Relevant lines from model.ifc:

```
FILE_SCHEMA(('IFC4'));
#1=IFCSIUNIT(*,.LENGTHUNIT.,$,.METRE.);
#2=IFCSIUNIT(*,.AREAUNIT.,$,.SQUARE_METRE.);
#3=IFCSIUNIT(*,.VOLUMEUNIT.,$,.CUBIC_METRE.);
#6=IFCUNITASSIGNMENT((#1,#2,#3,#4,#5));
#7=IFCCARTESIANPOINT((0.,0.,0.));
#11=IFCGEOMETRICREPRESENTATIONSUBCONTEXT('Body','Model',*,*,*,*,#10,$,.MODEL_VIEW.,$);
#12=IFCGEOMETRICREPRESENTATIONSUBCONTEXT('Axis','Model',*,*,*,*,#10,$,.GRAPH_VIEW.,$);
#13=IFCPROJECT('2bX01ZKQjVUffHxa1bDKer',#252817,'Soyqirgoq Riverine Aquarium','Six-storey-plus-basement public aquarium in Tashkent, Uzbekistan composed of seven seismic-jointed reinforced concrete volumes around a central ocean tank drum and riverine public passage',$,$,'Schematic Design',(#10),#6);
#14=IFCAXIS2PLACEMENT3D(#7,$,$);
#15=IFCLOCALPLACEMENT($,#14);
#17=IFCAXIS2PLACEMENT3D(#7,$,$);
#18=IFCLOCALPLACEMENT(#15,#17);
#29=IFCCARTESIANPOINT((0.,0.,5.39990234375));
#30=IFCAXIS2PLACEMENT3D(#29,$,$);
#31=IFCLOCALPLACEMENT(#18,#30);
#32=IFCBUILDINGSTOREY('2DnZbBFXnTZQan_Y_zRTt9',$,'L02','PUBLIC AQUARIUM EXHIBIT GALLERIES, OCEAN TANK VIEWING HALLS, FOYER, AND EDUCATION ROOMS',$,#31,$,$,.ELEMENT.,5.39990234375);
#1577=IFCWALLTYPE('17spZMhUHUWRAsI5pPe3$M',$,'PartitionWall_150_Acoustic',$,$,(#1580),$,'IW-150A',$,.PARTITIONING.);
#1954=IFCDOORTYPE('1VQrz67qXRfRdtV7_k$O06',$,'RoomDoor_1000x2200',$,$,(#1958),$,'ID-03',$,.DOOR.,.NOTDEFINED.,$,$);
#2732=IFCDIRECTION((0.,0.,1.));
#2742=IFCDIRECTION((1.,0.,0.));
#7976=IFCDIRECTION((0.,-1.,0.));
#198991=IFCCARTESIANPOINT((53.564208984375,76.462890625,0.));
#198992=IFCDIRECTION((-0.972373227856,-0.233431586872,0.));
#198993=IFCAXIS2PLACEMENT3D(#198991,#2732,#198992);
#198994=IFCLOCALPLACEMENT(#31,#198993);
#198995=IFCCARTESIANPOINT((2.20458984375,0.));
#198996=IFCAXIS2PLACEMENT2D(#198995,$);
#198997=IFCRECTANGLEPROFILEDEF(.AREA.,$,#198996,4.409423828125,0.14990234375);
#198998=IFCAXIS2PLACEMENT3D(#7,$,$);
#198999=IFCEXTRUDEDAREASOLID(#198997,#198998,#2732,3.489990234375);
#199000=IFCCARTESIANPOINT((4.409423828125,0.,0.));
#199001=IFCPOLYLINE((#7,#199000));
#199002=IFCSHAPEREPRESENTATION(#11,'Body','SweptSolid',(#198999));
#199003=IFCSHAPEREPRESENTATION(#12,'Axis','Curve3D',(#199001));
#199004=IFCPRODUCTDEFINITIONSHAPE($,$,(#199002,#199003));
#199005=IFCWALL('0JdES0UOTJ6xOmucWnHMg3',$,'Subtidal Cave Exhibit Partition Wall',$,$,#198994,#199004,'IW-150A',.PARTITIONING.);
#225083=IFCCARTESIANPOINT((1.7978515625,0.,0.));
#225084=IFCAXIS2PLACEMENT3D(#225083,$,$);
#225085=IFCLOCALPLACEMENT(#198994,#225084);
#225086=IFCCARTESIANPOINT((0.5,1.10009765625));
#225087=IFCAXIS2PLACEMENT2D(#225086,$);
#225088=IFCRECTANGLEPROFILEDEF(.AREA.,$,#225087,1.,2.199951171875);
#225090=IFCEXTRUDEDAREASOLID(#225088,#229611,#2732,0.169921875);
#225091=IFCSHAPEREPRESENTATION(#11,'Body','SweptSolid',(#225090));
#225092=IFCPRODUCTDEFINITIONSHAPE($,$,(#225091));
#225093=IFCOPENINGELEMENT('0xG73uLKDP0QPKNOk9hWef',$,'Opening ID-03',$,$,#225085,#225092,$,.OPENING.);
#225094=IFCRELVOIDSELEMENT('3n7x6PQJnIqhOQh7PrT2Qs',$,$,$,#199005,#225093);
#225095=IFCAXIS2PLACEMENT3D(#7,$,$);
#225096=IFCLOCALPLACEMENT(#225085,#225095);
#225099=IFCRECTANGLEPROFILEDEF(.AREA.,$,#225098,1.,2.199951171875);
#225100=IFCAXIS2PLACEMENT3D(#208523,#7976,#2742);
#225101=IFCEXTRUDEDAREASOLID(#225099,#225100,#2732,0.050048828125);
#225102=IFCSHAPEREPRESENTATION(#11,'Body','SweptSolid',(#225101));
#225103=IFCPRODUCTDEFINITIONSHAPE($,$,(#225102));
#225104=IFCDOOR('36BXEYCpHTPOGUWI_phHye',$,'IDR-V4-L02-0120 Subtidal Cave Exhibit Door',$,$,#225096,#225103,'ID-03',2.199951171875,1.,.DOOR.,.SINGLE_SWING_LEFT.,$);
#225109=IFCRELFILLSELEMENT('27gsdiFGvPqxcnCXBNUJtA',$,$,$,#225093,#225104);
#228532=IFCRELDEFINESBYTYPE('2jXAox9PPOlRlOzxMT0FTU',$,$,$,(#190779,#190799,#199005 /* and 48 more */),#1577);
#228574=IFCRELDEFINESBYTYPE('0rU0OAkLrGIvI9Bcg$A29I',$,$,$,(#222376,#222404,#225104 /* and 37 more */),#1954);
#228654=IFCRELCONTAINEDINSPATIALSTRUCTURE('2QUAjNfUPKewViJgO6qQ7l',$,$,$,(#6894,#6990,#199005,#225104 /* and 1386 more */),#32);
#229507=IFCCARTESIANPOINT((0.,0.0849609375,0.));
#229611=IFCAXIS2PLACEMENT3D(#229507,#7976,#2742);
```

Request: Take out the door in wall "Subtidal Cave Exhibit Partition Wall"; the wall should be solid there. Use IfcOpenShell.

```python
import ifcopenshell
import ifcopenshell.api.feature
import ifcopenshell.api.root
import ifcopenshell.geom
import ifcopenshell.util.shape

model = ifcopenshell.open("model.ifc")
settings = ifcopenshell.geom.settings()


def volume(element):
    """Net volume in cubic metres, openings subtracted."""
    shape = ifcopenshell.geom.create_shape(settings, element)
    return ifcopenshell.util.shape.get_volume(shape.geometry)


door = model.by_id(225104)
opening = door.FillsVoids[0].RelatingOpeningElement
wall = opening.VoidsElements[0].RelatingBuildingElement
before = volume(wall)

ifcopenshell.api.root.remove_product(model, product=door)
ifcopenshell.api.feature.remove_feature(model, feature=opening)

after = volume(wall)

print(f"wall volume {before:.3f} -> {after:.3f} m3")

model.write("model_updated.ifc")
```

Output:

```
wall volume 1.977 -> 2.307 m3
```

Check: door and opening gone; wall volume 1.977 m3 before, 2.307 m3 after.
